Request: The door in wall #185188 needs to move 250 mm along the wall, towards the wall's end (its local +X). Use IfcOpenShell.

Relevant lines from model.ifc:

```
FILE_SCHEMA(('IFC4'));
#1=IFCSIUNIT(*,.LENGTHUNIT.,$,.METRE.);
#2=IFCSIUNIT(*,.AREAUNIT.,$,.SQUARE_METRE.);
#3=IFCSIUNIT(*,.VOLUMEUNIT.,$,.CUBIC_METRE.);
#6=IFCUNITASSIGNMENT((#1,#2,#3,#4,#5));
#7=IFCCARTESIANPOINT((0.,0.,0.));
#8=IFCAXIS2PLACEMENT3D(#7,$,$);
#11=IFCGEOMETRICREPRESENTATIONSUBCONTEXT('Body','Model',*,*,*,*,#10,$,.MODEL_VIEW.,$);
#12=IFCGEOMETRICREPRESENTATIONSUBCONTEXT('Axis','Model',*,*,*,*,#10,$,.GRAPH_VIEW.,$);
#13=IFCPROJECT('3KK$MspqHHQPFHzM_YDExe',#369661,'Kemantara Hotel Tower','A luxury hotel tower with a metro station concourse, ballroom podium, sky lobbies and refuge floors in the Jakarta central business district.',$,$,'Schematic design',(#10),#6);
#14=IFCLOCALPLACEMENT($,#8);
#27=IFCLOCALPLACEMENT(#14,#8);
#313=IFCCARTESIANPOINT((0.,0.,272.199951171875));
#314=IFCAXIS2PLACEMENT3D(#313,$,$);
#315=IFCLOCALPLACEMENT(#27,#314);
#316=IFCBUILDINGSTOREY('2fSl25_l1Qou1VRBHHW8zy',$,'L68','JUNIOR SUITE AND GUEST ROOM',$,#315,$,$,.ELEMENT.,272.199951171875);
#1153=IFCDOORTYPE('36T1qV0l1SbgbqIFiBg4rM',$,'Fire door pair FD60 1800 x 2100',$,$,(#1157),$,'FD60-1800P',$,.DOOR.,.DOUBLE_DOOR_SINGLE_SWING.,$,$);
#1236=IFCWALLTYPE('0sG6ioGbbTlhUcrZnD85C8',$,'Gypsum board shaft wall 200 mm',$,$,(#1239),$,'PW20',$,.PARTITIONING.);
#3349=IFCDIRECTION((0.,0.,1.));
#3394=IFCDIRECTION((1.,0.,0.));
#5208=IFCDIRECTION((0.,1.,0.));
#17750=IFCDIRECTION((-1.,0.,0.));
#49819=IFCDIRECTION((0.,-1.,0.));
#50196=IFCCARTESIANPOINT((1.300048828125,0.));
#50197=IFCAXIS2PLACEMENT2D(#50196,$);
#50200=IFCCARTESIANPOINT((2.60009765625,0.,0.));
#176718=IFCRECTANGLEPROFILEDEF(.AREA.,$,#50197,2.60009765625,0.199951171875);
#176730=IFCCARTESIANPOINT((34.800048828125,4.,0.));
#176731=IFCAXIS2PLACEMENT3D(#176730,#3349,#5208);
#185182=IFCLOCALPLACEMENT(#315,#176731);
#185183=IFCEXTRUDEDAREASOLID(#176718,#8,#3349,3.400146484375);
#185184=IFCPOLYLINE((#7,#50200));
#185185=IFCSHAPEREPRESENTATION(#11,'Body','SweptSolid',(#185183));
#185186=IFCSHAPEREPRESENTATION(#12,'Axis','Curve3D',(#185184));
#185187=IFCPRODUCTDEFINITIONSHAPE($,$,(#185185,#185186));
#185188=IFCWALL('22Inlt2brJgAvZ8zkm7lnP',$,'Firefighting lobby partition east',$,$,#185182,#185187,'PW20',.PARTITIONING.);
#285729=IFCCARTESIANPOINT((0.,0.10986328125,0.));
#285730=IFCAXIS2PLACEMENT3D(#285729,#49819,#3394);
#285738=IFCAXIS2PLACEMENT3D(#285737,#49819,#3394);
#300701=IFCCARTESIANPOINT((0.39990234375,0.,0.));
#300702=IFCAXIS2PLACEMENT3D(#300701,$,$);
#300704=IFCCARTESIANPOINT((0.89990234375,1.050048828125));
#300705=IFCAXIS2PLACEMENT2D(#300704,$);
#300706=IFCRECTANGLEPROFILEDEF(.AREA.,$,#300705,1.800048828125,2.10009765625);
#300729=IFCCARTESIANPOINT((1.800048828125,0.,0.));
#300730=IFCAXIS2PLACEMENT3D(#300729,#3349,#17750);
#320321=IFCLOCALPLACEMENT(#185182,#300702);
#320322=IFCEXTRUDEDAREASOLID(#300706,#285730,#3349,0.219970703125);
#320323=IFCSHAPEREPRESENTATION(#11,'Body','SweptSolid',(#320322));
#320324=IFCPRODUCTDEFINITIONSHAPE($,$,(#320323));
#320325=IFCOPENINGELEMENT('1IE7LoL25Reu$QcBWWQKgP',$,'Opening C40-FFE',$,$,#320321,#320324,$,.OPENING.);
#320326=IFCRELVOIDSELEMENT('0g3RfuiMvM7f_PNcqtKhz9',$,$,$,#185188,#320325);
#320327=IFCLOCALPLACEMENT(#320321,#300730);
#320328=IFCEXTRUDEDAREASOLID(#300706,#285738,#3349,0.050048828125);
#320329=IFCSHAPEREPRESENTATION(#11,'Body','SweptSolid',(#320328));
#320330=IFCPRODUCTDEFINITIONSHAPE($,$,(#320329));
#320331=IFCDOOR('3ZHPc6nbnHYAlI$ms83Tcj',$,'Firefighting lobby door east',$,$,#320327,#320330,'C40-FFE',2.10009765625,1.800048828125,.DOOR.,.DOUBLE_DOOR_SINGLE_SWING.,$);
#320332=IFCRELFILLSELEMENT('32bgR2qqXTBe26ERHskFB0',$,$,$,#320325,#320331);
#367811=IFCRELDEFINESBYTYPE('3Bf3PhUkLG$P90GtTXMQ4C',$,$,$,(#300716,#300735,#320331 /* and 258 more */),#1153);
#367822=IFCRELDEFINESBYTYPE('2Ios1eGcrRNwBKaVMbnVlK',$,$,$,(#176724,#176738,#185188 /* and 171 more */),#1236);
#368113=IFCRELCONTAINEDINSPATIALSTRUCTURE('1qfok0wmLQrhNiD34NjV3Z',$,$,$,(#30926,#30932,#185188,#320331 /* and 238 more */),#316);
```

```python
import ifcopenshell
import ifcopenshell.api.geometry
import ifcopenshell.util.placement
import ifcopenshell.util.unit

model = ifcopenshell.open("model.ifc")
unit_scale = ifcopenshell.util.unit.calculate_unit_scale(model)

door = model.by_guid("3ZHPc6nbnHYAlI$ms83Tcj")
opening = door.FillsVoids[0].RelatingOpeningElement
wall = opening.VoidsElements[0].RelatingBuildingElement

wall_matrix = ifcopenshell.util.placement.get_local_placement(wall.ObjectPlacement)
shift = wall_matrix[:3, 0] * 0.25 / unit_scale
before = ifcopenshell.util.placement.get_local_placement(door.ObjectPlacement)[:3, 3].copy()

# The door is placed relative to its opening, so it follows when the opening moves.
matrix = ifcopenshell.util.placement.get_local_placement(opening.ObjectPlacement)
matrix[:3, 3] += shift
ifcopenshell.api.geometry.edit_object_placement(
    model, product=opening, matrix=matrix, is_si=False, should_transform_children=True
)

after = ifcopenshell.util.placement.get_local_placement(door.ObjectPlacement)[:3, 3]
print("door moved by", (after - before).round(3) + 0.0)

model.write("model_edited.ifc")
```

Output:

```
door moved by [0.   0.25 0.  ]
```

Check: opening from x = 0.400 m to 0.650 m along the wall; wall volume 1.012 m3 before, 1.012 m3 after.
